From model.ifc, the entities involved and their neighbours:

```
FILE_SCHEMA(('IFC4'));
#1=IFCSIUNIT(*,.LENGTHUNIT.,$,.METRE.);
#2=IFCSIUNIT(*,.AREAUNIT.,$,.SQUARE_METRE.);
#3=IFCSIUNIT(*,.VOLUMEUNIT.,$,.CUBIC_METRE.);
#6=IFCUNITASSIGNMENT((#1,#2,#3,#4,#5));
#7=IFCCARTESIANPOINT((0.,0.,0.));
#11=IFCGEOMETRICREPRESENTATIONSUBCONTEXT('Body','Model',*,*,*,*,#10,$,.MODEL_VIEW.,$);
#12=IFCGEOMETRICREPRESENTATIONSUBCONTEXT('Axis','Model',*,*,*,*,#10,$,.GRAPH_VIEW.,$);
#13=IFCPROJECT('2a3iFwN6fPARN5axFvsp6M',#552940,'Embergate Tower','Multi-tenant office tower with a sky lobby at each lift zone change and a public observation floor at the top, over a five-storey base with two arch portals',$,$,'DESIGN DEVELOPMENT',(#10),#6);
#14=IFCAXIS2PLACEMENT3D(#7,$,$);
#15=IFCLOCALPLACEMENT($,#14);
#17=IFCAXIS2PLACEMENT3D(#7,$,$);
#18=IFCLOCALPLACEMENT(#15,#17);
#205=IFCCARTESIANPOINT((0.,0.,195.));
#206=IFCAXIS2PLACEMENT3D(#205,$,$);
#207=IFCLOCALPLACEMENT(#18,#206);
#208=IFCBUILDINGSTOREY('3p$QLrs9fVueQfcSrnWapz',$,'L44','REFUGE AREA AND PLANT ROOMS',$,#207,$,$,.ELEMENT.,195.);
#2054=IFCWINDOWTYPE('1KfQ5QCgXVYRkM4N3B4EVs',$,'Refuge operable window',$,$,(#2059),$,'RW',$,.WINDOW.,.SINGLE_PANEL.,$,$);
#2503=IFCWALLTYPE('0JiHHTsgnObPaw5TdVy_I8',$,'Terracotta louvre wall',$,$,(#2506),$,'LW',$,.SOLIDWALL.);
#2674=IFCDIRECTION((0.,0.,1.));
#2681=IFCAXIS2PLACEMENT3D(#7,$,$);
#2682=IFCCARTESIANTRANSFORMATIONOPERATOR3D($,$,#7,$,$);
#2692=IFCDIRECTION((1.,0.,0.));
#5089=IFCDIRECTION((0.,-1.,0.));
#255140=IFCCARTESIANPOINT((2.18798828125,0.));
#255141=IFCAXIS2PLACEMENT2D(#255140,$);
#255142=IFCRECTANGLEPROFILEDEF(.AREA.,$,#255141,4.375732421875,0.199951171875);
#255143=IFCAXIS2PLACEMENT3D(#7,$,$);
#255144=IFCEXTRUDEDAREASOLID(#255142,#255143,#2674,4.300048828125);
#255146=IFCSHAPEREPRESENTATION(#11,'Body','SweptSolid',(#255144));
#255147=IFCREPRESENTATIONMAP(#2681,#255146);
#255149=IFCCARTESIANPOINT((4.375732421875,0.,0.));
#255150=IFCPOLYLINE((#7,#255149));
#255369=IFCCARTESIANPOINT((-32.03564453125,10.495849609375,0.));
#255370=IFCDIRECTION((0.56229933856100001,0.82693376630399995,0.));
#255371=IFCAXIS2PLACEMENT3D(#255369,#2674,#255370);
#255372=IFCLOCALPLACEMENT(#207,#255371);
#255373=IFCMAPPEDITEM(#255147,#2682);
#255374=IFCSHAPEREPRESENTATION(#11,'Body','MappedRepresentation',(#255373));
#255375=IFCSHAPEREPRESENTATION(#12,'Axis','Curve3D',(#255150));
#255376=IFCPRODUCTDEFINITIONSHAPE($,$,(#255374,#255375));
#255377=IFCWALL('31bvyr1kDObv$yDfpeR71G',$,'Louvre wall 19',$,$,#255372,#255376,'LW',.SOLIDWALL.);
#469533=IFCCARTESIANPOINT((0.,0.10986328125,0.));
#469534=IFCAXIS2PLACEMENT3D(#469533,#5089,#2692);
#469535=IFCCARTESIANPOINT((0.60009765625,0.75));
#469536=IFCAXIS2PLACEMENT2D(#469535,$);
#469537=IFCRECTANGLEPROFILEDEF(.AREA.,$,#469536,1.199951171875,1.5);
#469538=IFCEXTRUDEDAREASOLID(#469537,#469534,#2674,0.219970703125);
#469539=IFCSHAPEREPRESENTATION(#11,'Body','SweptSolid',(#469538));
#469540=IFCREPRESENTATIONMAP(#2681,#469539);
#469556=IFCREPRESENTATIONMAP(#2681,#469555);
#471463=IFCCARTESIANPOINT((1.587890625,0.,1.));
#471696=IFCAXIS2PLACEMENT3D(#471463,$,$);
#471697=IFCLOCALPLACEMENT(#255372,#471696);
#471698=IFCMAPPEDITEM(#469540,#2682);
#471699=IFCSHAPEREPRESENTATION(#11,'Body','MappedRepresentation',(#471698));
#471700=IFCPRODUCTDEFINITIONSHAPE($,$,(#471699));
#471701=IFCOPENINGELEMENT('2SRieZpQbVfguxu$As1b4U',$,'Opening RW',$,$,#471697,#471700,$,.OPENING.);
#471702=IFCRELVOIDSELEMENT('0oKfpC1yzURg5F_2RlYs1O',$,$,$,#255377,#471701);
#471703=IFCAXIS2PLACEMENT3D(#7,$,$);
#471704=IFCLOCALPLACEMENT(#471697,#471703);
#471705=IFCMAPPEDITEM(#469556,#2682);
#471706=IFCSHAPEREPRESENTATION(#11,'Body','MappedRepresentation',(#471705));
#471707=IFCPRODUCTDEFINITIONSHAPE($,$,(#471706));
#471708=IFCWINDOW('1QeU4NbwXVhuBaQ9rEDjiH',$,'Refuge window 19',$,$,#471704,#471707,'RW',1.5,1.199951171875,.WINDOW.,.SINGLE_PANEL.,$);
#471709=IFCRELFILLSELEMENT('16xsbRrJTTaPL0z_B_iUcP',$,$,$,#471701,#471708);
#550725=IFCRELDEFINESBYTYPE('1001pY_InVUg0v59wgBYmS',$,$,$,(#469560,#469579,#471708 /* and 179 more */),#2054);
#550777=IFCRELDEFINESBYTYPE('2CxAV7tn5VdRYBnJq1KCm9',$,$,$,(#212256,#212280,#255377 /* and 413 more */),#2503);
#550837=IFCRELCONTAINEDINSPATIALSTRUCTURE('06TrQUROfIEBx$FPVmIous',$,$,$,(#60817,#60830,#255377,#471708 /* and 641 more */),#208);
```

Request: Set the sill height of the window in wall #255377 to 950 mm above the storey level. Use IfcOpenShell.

```python
import numpy as np
import ifcopenshell
import ifcopenshell.api.geometry
import ifcopenshell.geom
import ifcopenshell.util.element
import ifcopenshell.util.placement
import ifcopenshell.util.shape
import ifcopenshell.util.unit

model = ifcopenshell.open("model.ifc")
unit_scale = ifcopenshell.util.unit.calculate_unit_scale(model)

window = model.by_id(471708)
opening = window.FillsVoids[0].RelatingOpeningElement
storey = ifcopenshell.util.element.get_container(window, ifc_class="IfcBuildingStorey")
level = ifcopenshell.util.placement.get_local_placement(storey.ObjectPlacement)[2, 3]

# The opening's origin need not be at the sill, so measure its lowest point.
shape = ifcopenshell.geom.create_shape(ifcopenshell.geom.settings(), opening)
bottom = ifcopenshell.util.shape.get_shape_bottom_elevation(shape, shape.geometry) / unit_scale
dz = level + 0.95 / unit_scale - bottom

shift = np.array([0.0, 0.0, dz])
# The window is placed relative to its opening, so it follows when the opening moves.
matrix = ifcopenshell.util.placement.get_local_placement(opening.ObjectPlacement)
matrix[:3, 3] += shift
ifcopenshell.api.geometry.edit_object_placement(
    model, product=opening, matrix=matrix, is_si=False, should_transform_children=True
)

print(f"moved by {dz * unit_scale:+.3f} m")

model.write("model_edited.ifc")
```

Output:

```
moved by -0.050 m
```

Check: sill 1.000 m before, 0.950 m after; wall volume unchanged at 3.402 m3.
